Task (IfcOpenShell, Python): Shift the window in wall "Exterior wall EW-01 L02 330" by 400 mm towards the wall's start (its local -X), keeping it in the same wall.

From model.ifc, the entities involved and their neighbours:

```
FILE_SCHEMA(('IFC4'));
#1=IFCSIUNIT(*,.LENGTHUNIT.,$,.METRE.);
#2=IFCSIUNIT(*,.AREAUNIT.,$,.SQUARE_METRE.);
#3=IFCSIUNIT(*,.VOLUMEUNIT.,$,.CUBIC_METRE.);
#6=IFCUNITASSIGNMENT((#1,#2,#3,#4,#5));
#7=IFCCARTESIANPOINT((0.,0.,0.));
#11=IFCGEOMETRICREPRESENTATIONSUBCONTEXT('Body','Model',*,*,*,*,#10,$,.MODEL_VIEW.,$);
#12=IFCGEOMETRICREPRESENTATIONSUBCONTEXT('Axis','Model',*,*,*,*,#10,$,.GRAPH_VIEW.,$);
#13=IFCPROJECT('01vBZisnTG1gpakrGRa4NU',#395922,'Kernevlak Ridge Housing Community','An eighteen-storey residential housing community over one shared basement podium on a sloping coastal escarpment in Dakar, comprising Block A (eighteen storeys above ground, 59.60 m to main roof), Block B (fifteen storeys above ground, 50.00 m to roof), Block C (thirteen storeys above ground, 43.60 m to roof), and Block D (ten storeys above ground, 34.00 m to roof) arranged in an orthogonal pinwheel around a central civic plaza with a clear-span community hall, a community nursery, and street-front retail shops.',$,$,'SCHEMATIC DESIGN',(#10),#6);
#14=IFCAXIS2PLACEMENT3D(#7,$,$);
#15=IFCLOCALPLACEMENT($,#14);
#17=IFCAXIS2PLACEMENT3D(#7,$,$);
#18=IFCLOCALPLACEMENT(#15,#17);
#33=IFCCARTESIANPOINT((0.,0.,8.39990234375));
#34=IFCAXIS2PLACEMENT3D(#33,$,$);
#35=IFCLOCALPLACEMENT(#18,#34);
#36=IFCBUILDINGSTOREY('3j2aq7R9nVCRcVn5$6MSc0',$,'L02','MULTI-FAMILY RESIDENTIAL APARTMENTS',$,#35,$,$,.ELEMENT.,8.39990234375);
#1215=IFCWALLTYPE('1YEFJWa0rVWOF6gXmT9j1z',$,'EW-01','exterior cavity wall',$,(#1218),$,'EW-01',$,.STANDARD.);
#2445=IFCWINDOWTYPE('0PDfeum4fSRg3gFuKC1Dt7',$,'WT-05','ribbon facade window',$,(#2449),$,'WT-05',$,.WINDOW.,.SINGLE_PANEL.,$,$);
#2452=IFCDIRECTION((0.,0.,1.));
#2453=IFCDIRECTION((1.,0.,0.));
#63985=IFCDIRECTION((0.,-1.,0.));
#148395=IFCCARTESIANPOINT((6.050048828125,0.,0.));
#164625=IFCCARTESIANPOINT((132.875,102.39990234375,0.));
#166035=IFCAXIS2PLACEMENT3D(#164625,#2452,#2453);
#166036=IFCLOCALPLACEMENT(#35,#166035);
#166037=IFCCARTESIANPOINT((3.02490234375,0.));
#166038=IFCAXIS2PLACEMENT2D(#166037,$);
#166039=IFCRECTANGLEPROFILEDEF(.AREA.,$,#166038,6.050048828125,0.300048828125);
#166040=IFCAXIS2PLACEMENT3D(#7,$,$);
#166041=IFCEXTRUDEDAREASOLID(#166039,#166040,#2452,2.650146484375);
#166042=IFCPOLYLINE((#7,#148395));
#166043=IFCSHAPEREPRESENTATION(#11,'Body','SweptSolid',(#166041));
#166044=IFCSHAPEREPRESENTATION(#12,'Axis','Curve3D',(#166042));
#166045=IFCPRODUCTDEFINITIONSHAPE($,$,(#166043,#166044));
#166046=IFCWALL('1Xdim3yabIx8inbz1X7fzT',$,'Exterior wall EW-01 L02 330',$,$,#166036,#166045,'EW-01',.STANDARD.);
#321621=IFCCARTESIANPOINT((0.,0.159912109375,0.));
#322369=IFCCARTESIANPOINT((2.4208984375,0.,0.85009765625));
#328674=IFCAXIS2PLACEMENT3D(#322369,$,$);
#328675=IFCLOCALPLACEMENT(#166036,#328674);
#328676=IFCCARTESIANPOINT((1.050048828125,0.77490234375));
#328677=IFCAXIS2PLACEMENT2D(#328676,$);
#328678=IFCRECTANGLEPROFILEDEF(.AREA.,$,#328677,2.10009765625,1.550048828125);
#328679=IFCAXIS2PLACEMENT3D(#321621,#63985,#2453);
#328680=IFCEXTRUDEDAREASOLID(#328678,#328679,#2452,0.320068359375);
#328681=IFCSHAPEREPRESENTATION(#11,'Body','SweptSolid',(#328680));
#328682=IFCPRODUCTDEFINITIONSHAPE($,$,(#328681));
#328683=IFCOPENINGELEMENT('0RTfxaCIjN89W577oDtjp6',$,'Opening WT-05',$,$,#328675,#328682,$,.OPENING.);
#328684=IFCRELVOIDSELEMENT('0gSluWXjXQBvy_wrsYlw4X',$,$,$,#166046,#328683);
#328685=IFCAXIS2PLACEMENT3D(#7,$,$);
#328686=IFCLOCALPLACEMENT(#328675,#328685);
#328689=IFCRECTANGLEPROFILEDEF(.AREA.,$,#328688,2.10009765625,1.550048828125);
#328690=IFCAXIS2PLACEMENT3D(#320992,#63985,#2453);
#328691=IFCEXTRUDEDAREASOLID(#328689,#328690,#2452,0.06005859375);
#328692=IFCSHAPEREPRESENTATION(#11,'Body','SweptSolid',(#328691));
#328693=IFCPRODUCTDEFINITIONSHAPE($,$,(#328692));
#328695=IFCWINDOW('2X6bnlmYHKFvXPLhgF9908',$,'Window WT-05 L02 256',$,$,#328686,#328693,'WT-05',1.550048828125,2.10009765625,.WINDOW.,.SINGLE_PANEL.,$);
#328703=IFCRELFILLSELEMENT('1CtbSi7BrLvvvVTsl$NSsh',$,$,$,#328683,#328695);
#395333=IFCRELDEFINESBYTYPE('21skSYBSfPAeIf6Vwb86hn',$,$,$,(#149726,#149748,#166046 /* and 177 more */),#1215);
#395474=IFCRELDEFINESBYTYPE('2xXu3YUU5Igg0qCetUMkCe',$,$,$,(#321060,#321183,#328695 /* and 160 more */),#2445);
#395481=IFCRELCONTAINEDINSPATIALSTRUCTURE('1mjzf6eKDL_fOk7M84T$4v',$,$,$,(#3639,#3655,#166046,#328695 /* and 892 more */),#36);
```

```python
import ifcopenshell
import ifcopenshell.api.geometry
import ifcopenshell.util.placement
import ifcopenshell.util.unit

model = ifcopenshell.open("model.ifc")
unit_scale = ifcopenshell.util.unit.calculate_unit_scale(model)

window = model.by_guid("2X6bnlmYHKFvXPLhgF9908")
opening = window.FillsVoids[0].RelatingOpeningElement
wall = opening.VoidsElements[0].RelatingBuildingElement

wall_matrix = ifcopenshell.util.placement.get_local_placement(wall.ObjectPlacement)
shift = wall_matrix[:3, 0] * -0.4 / unit_scale
before = ifcopenshell.util.placement.get_local_placement(window.ObjectPlacement)[:3, 3].copy()

# The window is placed relative to its opening, so it follows when the opening moves.
matrix = ifcopenshell.util.placement.get_local_placement(opening.ObjectPlacement)
matrix[:3, 3] += shift
ifcopenshell.api.geometry.edit_object_placement(
    model, product=opening, matrix=matrix, is_si=False, should_transform_children=True
)

after = ifcopenshell.util.placement.get_local_placement(window.ObjectPlacement)[:3, 3]
print("window moved by", (after - before).round(3) + 0.0)

model.write("model_updated.ifc")
```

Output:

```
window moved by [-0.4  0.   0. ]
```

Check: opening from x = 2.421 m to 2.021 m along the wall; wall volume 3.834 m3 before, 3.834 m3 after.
